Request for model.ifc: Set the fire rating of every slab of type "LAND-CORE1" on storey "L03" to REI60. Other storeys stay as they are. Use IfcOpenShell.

First a look at what the model holds.

```python
import ifcopenshell
import ifcopenshell.util.element

model = ifcopenshell.open("model.ifc")
print(model.schema)
storey = next(s for s in model.by_type("IfcBuildingStorey") if s.Name == "L03")
slabs = [e for e in ifcopenshell.util.element.get_decomposition(storey) if e.is_a("IfcSlab")]
seen = {}
for e in slabs:
    element_type = ifcopenshell.util.element.get_type(e)
    key = (element_type.Name if element_type != e and element_type else None, ifcopenshell.util.element.get_pset(e, "Pset_SlabCommon", "FireRating"))
    seen[key] = seen.get(key, 0) + 1
for (name, value), count in sorted(seen.items(), key=str):
    print(count, "x", name, "|", value)
```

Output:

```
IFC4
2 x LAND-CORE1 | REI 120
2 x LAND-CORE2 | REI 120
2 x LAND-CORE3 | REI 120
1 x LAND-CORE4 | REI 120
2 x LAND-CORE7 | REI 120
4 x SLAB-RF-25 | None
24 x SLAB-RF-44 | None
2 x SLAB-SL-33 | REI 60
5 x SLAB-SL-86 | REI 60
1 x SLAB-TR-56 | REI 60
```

```python
import ifcopenshell
import ifcopenshell.api.pset
import ifcopenshell.util.element

model = ifcopenshell.open("model.ifc")

storey = next(s for s in model.by_type("IfcBuildingStorey") if s.Name == "L03")
slabs = [e for e in ifcopenshell.util.element.get_decomposition(storey) if e.is_a("IfcSlab")]

count = 0
for e in slabs:
    element_type = ifcopenshell.util.element.get_type(e)
    if element_type in (None, e) or element_type.Name != "LAND-CORE1":
        continue
    # add_pset returns the element's existing set when there is one.
    pset = ifcopenshell.api.pset.add_pset(model, product=e, name="Pset_SlabCommon")
    ifcopenshell.api.pset.edit_pset(model, pset=pset, properties={"FireRating": "REI60"})
    count += 1

print(count, "slabs updated")

model.write("model-out.ifc")
```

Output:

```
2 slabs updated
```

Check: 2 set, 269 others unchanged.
